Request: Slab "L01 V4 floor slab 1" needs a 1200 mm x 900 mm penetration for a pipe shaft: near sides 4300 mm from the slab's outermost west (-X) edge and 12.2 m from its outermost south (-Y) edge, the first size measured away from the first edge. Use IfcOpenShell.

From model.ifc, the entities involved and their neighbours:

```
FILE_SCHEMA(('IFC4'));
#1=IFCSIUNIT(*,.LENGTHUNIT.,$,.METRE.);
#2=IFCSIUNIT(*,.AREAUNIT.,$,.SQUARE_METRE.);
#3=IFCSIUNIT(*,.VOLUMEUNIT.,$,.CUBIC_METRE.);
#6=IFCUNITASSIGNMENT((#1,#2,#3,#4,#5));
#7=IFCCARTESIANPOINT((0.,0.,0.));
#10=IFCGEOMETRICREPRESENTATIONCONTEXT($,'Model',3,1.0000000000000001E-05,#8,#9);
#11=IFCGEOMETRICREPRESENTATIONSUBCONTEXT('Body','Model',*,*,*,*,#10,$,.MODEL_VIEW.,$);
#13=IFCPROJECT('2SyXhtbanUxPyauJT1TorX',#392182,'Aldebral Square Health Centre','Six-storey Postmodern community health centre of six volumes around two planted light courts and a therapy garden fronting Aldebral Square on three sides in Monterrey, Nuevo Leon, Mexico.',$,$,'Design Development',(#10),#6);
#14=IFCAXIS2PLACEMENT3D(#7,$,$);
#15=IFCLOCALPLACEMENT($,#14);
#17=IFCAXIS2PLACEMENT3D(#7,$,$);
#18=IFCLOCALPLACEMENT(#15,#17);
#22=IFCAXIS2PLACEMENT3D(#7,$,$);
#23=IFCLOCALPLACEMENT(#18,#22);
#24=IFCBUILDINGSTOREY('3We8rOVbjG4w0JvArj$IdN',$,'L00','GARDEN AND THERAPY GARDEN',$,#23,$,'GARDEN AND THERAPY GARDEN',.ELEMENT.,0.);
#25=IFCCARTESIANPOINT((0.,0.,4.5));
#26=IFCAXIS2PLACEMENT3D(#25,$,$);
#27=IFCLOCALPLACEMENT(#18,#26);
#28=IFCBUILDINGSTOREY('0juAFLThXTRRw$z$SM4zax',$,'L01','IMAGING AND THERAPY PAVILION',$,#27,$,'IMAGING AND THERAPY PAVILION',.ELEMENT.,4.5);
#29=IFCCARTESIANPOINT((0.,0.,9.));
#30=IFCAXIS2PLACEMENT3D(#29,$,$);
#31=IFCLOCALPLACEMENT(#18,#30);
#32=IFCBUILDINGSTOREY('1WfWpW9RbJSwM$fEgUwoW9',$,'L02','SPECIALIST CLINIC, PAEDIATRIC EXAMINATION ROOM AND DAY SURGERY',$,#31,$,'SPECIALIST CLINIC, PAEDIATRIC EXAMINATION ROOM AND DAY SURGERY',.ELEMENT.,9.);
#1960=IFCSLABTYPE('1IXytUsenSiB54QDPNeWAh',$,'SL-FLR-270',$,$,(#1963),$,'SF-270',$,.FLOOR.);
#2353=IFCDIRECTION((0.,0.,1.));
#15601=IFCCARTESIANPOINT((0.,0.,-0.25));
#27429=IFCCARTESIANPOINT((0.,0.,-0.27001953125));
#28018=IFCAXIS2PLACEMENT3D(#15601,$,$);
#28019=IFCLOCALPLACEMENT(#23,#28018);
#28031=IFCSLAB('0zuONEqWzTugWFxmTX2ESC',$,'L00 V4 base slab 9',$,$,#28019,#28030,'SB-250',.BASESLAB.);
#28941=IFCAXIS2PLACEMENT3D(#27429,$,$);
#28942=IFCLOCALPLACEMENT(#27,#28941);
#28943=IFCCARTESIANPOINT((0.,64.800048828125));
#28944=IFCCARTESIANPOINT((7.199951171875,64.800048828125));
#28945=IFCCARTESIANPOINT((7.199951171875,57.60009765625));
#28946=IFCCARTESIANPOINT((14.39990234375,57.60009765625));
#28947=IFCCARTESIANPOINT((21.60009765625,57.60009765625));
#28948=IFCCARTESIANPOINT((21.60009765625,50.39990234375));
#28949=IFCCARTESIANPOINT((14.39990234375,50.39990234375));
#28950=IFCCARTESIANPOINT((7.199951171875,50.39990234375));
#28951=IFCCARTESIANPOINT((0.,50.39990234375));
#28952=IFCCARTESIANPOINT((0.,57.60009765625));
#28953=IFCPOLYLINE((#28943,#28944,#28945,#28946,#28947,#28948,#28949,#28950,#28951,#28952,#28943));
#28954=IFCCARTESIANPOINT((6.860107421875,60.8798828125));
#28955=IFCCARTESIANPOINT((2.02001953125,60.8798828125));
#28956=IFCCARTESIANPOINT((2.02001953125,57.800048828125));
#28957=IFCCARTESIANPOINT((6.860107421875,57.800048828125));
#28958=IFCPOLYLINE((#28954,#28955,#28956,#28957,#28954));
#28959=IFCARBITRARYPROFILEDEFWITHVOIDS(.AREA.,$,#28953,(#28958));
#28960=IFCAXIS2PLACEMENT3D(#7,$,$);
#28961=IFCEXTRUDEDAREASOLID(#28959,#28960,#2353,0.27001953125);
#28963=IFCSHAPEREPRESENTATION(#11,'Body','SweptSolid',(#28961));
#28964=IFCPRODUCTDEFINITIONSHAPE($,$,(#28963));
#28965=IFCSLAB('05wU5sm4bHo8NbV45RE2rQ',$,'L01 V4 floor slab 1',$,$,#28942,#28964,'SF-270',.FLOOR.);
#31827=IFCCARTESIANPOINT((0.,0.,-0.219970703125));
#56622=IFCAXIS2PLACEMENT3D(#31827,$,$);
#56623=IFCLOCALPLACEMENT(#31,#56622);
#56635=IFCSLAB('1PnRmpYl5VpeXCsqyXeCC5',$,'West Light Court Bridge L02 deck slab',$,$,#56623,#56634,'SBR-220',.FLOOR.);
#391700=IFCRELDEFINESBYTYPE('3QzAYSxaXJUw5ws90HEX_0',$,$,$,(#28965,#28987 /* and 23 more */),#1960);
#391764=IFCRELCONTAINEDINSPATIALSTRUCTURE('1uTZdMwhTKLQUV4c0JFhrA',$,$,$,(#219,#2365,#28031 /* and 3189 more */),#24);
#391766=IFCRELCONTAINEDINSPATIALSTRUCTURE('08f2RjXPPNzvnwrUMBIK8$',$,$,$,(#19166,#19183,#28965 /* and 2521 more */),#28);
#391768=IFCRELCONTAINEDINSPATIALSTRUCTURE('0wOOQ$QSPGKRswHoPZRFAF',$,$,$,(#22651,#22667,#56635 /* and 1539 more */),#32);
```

```python
import numpy as np
import ifcopenshell
import ifcopenshell.api.feature
import ifcopenshell.api.geometry
import ifcopenshell.api.root
import ifcopenshell.geom
import ifcopenshell.util.placement
import ifcopenshell.util.representation
import ifcopenshell.util.shape
import ifcopenshell.util.unit

model = ifcopenshell.open("model.ifc")
unit_scale = ifcopenshell.util.unit.calculate_unit_scale(model)
settings = ifcopenshell.geom.settings()


def volume(element):
    """Net volume in cubic metres, openings subtracted."""
    shape = ifcopenshell.geom.create_shape(settings, element)
    return ifcopenshell.util.shape.get_volume(shape.geometry)


slab = model.by_guid("05wU5sm4bHo8NbV45RE2rQ")
before = volume(slab)

# Extent in the slab's own axes, in metres. The edges named are its -X and -Y sides.
slab_shape = ifcopenshell.geom.create_shape(settings, slab)
vertices = ifcopenshell.util.shape.get_vertices(slab_shape.geometry)
x_min, y_min, bottom = vertices.min(axis=0)
top = vertices[:, 2].max()

opening = ifcopenshell.api.root.create_entity(model, ifc_class="IfcOpeningElement", name="Pipe shaft opening", predefined_type="OPENING")
context = ifcopenshell.util.representation.get_context(model, "Model", "Body", "MODEL_VIEW")
width, depth = 1.2, 0.9
outline = [(0.0, 0.0), (width, 0.0), (width, depth), (0.0, depth), (0.0, 0.0)]
# Overshoot both faces by 50 mm so the cut is clean.
shape = ifcopenshell.api.geometry.add_slab_representation(
    model, context=context, depth=top - bottom + 0.1, polyline=outline
)
ifcopenshell.api.geometry.assign_representation(model, product=opening, representation=shape)

matrix = ifcopenshell.util.placement.get_local_placement(slab.ObjectPlacement)
matrix[:, 3] = matrix @ np.append(np.array([x_min + 4.3, y_min + 12.2, bottom - 0.05]) / unit_scale, 1.0)
ifcopenshell.api.geometry.edit_object_placement(model, product=opening, matrix=matrix, is_si=False)
ifcopenshell.api.feature.add_feature(model, feature=opening, element=slab)

after = volume(slab)

print(f"slab volume {before:.3f} -> {after:.3f} m3")

model.write("model-out.ifc")
```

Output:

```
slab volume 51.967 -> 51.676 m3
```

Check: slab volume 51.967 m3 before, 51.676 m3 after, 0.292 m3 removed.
